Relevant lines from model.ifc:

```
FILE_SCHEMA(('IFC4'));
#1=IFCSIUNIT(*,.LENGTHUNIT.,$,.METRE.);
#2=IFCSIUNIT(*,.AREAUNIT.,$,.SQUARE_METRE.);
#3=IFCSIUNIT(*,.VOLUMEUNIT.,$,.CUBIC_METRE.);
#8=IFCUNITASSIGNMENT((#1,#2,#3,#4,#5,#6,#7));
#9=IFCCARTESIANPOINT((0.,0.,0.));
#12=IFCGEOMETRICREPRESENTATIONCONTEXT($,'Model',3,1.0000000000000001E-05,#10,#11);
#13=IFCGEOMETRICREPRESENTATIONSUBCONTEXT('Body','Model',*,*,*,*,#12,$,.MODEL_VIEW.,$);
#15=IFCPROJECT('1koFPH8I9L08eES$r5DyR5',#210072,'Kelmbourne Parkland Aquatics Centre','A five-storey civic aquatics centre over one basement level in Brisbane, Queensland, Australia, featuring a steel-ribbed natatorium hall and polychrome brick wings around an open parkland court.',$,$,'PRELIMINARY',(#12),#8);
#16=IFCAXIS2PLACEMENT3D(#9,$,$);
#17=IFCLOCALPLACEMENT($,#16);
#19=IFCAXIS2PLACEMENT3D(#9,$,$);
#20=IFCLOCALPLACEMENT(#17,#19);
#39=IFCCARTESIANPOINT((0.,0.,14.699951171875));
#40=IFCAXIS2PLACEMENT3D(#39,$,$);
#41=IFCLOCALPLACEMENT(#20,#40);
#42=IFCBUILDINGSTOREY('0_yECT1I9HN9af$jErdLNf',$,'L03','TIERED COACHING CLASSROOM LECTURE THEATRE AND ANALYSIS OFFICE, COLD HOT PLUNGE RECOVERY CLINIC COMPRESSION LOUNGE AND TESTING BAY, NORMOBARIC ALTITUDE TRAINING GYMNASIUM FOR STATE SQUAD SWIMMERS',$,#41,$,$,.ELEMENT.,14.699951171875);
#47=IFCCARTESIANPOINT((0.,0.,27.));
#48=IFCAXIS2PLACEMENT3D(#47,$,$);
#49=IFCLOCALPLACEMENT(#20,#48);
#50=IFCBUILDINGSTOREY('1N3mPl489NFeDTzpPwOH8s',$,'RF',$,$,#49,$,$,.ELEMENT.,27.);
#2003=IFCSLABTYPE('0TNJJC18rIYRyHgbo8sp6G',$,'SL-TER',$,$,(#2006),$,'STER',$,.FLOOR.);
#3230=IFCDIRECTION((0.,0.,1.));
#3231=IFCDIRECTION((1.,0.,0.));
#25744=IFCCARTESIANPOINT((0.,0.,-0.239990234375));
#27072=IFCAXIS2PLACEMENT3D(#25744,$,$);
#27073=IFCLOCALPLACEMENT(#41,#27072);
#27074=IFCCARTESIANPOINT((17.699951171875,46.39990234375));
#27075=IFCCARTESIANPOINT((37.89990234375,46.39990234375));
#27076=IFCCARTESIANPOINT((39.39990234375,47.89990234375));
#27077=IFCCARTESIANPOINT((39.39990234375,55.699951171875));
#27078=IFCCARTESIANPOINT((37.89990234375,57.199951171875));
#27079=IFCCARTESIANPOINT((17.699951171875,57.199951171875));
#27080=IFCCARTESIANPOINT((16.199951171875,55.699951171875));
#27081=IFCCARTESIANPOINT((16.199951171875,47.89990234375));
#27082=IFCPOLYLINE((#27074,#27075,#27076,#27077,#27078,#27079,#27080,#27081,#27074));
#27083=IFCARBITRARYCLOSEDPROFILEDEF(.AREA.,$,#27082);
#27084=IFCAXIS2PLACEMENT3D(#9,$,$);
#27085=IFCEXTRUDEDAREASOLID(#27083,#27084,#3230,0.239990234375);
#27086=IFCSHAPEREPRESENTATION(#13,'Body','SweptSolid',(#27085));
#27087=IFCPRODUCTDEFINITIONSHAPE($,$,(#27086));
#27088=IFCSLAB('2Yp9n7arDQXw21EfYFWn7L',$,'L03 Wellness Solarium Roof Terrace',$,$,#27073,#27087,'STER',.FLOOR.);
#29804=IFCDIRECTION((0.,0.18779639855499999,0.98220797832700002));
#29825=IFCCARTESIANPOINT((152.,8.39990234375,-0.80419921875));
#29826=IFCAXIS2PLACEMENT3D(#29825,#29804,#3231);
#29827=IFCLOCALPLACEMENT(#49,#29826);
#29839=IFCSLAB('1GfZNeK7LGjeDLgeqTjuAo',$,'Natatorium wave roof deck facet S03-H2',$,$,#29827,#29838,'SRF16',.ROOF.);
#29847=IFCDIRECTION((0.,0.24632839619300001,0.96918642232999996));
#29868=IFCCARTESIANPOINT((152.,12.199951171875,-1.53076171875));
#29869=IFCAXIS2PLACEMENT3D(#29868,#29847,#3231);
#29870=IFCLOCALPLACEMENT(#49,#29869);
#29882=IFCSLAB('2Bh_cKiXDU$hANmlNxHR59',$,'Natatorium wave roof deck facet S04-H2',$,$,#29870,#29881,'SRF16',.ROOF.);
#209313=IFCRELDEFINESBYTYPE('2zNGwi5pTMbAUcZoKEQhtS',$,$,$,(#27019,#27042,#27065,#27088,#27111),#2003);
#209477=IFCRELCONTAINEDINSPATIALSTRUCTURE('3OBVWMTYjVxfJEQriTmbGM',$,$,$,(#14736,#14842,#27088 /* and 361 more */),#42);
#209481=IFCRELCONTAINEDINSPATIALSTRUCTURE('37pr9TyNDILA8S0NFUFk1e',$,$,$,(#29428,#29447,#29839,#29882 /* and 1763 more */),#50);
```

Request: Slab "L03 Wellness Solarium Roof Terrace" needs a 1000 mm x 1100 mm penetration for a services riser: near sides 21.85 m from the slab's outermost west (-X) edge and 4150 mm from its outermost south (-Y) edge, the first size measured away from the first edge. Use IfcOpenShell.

```python
import numpy as np
import ifcopenshell
import ifcopenshell.api.feature
import ifcopenshell.api.geometry
import ifcopenshell.api.root
import ifcopenshell.geom
import ifcopenshell.util.placement
import ifcopenshell.util.representation
import ifcopenshell.util.shape
import ifcopenshell.util.unit

model = ifcopenshell.open("model.ifc")
unit_scale = ifcopenshell.util.unit.calculate_unit_scale(model)
settings = ifcopenshell.geom.settings()


def volume(element):
    """Net volume in cubic metres, openings subtracted."""
    shape = ifcopenshell.geom.create_shape(settings, element)
    return ifcopenshell.util.shape.get_volume(shape.geometry)


slab = model.by_guid("2Yp9n7arDQXw21EfYFWn7L")
before = volume(slab)

# Extent in the slab's own axes, in metres. The edges named are its -X and -Y sides.
slab_shape = ifcopenshell.geom.create_shape(settings, slab)
vertices = ifcopenshell.util.shape.get_vertices(slab_shape.geometry)
x_min, y_min, bottom = vertices.min(axis=0)
top = vertices[:, 2].max()

opening = ifcopenshell.api.root.create_entity(model, ifc_class="IfcOpeningElement", name="Services riser opening", predefined_type="OPENING")
context = ifcopenshell.util.representation.get_context(model, "Model", "Body", "MODEL_VIEW")
width, depth = 1, 1.1
outline = [(0.0, 0.0), (width, 0.0), (width, depth), (0.0, depth), (0.0, 0.0)]
# Overshoot both faces by 50 mm so the cut is clean.
shape = ifcopenshell.api.geometry.add_slab_representation(
    model, context=context, depth=top - bottom + 0.1, polyline=outline
)
ifcopenshell.api.geometry.assign_representation(model, product=opening, representation=shape)

matrix = ifcopenshell.util.placement.get_local_placement(slab.ObjectPlacement)
matrix[:, 3] = matrix @ np.append(np.array([x_min + 21.85, y_min + 4.15, bottom - 0.05]) / unit_scale, 1.0)
ifcopenshell.api.geometry.edit_object_placement(model, product=opening, matrix=matrix, is_si=False)
ifcopenshell.api.feature.add_feature(model, feature=opening, element=slab)

after = volume(slab)

print(f"slab volume {before:.3f} -> {after:.3f} m3")

model.write("model_rev.ifc")
```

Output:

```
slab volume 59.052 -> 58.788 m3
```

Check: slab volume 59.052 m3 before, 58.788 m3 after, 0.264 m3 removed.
